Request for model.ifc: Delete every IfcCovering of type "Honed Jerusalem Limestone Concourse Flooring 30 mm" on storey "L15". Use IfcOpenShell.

First a look at what the model holds.

```python
import ifcopenshell
import ifcopenshell.util.element

model = ifcopenshell.open("model.ifc")
print(model.schema)
storey = next(s for s in model.by_type("IfcBuildingStorey") if s.Name == "L15")
coverings = [e for e in ifcopenshell.util.element.get_decomposition(storey) if e.is_a("IfcCovering")]
seen = {}
for e in coverings:
    element_type = ifcopenshell.util.element.get_type(e)
    name = element_type.Name if element_type not in (None, e) else None
    seen[name] = seen.get(name, 0) + 1
for name, count in sorted(seen.items(), key=str):
    print(count, "x", name)
```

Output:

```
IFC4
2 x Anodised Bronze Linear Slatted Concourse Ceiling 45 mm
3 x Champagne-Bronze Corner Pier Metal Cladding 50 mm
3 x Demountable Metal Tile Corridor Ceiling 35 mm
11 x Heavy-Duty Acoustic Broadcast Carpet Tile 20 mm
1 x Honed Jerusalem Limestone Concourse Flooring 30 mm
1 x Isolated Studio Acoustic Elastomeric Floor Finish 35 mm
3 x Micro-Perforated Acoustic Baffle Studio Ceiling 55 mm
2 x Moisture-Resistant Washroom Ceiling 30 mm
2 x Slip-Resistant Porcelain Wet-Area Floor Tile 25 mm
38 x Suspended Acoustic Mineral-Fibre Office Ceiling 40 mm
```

```python
import ifcopenshell
import ifcopenshell.api.root
import ifcopenshell.util.element

model = ifcopenshell.open("model.ifc")

storey = next(s for s in model.by_type("IfcBuildingStorey") if s.Name == "L15")
coverings = [e for e in ifcopenshell.util.element.get_decomposition(storey) if e.is_a("IfcCovering")]
targets = [e for e in coverings if (t := ifcopenshell.util.element.get_type(e)) not in (None, e) and t.Name == "Honed Jerusalem Limestone Concourse Flooring 30 mm"]

for e in targets:
    ifcopenshell.api.root.remove_product(model, product=e)
print(len(targets), "removed")

model.write("model-out.ifc")
```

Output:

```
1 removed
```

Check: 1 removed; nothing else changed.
